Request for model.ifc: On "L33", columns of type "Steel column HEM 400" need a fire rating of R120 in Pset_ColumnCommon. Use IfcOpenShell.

First a look at what the model holds.

```python
import ifcopenshell
import ifcopenshell.util.element

model = ifcopenshell.open("model.ifc")
print(model.schema)
storey = next(s for s in model.by_type("IfcBuildingStorey") if s.Name == "L33")
columns = [e for e in ifcopenshell.util.element.get_decomposition(storey) if e.is_a("IfcColumn")]
seen = {}
for e in columns:
    element_type = ifcopenshell.util.element.get_type(e)
    key = (element_type.Name if element_type != e and element_type else None, ifcopenshell.util.element.get_pset(e, "Pset_ColumnCommon", "FireRating"))
    seen[key] = seen.get(key, 0) + 1
for (name, value), count in sorted(seen.items(), key=str):
    print(count, "x", name, "|", value)
```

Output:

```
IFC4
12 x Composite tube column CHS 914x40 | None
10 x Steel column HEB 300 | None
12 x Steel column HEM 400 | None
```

```python
import ifcopenshell
import ifcopenshell.api.pset
import ifcopenshell.util.element

model = ifcopenshell.open("model.ifc")

storey = next(s for s in model.by_type("IfcBuildingStorey") if s.Name == "L33")
columns = [e for e in ifcopenshell.util.element.get_decomposition(storey) if e.is_a("IfcColumn")]

count = 0
for e in columns:
    element_type = ifcopenshell.util.element.get_type(e)
    if element_type in (None, e) or element_type.Name != "Steel column HEM 400":
        continue
    found = ifcopenshell.util.element.get_pset(e, "Pset_ColumnCommon", should_inherit=False)
    if found:
        pset = model.by_id(found["id"])
        if len(ifcopenshell.util.element.get_elements_by_pset(pset)) > 1:
            pset = ifcopenshell.api.pset.unshare_pset(model, products=[e], pset=pset)[0]
    else:
        pset = ifcopenshell.api.pset.add_pset(model, product=e, name="Pset_ColumnCommon")
    ifcopenshell.api.pset.edit_pset(model, pset=pset, properties={"FireRating": "R120"})
    count += 1

print(count, "columns updated")

model.write("model_edited.ifc")
```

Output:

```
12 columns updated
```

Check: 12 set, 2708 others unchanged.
